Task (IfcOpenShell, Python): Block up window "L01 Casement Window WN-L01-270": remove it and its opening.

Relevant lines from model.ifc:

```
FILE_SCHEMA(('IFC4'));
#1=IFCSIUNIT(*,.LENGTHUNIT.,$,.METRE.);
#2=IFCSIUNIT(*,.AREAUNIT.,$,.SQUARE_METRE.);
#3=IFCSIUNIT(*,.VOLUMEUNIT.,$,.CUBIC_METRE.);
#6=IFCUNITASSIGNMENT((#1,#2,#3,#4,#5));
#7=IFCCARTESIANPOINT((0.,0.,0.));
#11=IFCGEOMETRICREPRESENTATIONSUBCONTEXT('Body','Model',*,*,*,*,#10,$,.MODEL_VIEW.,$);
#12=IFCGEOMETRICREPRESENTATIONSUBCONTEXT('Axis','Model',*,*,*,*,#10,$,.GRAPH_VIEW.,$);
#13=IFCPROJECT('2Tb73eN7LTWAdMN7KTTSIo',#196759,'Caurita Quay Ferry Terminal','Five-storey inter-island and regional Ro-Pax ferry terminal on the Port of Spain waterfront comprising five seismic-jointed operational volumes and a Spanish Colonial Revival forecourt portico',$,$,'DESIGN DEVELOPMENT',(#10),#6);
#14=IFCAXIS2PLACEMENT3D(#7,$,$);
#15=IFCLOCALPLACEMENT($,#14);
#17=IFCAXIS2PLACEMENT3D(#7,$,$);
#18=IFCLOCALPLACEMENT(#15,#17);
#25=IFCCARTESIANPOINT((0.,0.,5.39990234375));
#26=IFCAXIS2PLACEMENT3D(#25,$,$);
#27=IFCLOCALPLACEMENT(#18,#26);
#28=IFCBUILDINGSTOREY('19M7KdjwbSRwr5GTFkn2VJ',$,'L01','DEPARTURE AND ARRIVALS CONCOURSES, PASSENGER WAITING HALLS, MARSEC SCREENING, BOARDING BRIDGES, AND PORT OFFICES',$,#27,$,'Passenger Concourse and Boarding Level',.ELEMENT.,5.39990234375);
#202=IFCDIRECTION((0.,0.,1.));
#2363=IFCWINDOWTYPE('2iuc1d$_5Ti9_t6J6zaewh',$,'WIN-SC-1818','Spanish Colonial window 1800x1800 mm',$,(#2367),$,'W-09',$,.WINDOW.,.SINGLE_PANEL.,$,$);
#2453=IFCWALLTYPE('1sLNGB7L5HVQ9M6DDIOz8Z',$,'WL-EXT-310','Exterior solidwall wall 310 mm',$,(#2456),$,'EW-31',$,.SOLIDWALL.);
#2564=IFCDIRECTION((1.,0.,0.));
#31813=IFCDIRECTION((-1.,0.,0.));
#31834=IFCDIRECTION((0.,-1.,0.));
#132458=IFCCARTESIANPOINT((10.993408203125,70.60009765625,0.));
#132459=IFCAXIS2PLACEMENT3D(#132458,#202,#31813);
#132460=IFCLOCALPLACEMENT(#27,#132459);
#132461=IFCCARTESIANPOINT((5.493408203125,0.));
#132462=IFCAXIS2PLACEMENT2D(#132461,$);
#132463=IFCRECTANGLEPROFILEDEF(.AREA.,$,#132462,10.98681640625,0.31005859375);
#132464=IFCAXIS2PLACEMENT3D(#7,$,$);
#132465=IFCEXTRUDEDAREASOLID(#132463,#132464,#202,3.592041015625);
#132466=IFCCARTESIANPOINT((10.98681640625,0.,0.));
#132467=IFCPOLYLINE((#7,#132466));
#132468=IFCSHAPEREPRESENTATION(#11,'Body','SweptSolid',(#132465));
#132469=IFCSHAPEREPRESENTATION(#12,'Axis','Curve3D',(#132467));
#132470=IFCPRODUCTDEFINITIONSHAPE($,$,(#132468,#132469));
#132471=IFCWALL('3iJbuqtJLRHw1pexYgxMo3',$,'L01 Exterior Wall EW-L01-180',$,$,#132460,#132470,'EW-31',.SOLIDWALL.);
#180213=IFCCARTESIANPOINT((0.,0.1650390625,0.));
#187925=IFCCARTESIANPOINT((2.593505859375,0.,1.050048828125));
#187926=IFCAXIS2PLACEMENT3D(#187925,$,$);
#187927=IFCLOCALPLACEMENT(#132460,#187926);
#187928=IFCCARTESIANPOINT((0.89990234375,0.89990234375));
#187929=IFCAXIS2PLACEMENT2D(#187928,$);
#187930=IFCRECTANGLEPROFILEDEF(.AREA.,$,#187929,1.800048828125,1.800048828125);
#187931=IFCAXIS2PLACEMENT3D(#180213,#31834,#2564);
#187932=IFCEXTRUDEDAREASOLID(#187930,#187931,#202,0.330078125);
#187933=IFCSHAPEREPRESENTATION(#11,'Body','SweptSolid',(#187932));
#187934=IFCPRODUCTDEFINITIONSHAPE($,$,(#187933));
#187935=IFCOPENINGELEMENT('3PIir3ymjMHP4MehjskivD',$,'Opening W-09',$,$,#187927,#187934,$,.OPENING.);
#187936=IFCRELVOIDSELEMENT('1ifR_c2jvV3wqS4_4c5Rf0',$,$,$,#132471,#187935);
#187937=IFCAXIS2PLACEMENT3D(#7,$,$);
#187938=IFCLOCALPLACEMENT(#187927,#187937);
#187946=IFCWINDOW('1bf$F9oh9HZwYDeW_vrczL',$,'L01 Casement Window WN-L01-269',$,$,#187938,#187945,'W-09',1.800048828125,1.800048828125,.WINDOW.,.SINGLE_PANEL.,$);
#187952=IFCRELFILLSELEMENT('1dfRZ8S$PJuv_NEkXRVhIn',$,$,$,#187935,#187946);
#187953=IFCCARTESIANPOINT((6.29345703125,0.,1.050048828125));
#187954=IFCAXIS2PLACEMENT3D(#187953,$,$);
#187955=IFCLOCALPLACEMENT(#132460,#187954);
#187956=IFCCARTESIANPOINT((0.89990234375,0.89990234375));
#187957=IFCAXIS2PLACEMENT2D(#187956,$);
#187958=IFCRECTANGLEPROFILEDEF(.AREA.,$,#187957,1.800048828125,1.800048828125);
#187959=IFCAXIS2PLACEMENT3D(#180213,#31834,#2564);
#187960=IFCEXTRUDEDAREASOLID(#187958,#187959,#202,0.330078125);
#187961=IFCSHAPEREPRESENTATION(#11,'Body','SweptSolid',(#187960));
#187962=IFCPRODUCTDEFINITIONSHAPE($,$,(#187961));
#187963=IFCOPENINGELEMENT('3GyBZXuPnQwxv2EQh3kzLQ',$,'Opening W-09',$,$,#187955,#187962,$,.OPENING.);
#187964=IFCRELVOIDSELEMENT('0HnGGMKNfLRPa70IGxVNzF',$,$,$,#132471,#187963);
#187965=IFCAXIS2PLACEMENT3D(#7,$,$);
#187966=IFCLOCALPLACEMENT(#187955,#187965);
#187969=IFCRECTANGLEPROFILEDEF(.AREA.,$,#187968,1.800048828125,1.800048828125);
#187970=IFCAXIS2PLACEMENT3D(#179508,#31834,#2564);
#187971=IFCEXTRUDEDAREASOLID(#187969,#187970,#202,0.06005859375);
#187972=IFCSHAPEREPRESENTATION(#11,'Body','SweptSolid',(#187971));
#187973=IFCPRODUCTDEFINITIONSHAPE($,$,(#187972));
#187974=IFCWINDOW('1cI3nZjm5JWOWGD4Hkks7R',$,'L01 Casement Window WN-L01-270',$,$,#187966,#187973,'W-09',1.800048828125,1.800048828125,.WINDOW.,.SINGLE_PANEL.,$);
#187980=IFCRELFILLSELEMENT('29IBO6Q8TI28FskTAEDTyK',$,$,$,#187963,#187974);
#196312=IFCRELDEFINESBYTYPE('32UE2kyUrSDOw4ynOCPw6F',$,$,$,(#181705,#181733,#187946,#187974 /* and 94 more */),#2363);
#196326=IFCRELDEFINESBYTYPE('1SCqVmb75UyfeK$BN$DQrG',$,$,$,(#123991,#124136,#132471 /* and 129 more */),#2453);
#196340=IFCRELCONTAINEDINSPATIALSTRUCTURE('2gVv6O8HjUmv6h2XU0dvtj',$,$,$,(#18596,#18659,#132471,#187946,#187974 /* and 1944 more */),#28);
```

```python
import ifcopenshell
import ifcopenshell.api.feature
import ifcopenshell.api.root
import ifcopenshell.geom
import ifcopenshell.util.shape

model = ifcopenshell.open("model.ifc")
settings = ifcopenshell.geom.settings()


def volume(element):
    """Net volume in cubic metres, openings subtracted."""
    shape = ifcopenshell.geom.create_shape(settings, element)
    return ifcopenshell.util.shape.get_volume(shape.geometry)


window = model.by_guid("1cI3nZjm5JWOWGD4Hkks7R")
opening = window.FillsVoids[0].RelatingOpeningElement
wall = opening.VoidsElements[0].RelatingBuildingElement
before = volume(wall)

ifcopenshell.api.root.remove_product(model, product=window)
ifcopenshell.api.feature.remove_feature(model, feature=opening)

after = volume(wall)

print(f"wall volume {before:.3f} -> {after:.3f} m3")

model.write("model-out.ifc")
```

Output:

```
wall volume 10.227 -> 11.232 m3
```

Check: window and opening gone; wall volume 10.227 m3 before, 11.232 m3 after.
